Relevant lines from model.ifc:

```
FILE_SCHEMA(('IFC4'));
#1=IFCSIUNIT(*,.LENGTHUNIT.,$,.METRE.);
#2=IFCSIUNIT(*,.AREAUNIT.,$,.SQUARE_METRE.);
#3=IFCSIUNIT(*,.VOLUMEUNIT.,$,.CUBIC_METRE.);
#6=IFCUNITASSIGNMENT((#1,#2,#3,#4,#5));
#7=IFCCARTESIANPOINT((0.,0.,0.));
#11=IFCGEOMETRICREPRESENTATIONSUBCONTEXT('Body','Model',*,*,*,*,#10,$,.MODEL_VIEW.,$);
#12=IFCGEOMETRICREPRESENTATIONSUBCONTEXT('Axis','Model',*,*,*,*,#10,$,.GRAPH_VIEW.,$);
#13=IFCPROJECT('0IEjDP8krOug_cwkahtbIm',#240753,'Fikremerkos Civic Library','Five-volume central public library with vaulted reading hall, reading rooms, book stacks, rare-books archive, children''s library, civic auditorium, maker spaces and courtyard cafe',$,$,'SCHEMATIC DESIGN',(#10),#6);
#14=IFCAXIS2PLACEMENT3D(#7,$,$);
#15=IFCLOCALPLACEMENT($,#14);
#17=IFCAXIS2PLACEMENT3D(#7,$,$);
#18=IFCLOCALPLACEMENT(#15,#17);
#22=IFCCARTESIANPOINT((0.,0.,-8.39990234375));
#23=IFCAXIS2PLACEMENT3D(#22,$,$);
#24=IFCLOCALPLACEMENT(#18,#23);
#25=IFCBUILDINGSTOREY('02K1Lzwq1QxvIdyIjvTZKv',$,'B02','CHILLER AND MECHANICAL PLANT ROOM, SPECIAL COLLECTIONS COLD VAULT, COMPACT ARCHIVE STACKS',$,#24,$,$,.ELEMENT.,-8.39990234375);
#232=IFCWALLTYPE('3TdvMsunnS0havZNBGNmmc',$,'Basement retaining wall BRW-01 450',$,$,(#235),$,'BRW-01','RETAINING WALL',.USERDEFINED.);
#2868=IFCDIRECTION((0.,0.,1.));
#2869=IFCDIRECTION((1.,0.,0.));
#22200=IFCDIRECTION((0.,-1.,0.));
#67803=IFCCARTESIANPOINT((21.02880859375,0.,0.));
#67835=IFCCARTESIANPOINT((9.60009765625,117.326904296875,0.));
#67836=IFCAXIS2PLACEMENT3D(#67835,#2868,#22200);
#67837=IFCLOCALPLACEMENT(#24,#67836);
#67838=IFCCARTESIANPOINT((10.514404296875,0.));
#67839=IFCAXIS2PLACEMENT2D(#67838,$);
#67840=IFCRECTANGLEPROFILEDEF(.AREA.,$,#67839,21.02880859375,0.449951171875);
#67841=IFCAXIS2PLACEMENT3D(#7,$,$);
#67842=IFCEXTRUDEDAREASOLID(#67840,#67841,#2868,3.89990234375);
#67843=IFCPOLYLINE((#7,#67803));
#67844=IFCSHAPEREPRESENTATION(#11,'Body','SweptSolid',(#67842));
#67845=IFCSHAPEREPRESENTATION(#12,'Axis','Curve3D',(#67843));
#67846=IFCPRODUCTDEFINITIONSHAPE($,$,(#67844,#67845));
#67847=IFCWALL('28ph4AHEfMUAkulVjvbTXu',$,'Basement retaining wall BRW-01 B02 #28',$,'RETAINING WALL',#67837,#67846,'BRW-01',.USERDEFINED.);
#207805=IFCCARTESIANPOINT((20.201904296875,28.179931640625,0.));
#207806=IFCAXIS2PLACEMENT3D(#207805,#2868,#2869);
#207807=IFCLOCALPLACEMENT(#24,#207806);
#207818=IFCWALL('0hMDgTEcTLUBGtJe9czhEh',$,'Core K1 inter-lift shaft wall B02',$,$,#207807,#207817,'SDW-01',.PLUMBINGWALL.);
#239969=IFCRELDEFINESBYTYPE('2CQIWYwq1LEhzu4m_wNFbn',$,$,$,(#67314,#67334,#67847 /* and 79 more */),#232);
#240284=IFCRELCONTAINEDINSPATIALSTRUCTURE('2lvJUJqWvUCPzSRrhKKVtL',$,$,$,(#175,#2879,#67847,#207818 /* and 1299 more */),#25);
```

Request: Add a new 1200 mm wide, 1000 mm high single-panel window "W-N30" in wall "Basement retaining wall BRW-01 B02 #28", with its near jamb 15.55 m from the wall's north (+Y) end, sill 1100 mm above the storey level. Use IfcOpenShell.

```python
import numpy as np
import ifcopenshell
import ifcopenshell.api.feature
import ifcopenshell.api.geometry
import ifcopenshell.api.root
import ifcopenshell.api.spatial
import ifcopenshell.geom
import ifcopenshell.util.element
import ifcopenshell.util.placement
import ifcopenshell.util.representation
import ifcopenshell.util.shape
import ifcopenshell.util.unit

model = ifcopenshell.open("model.ifc")
unit_scale = ifcopenshell.util.unit.calculate_unit_scale(model)
settings = ifcopenshell.geom.settings()


def volume(element):
    """Net volume in cubic metres, openings subtracted."""
    shape = ifcopenshell.geom.create_shape(settings, element)
    return ifcopenshell.util.shape.get_volume(shape.geometry)


wall = model.by_guid("28ph4AHEfMUAkulVjvbTXu")
storey = ifcopenshell.util.element.get_container(wall, ifc_class="IfcBuildingStorey")
context = ifcopenshell.util.representation.get_context(model, "Model", "Body", "MODEL_VIEW")
before = volume(wall)

width, height, from_end, sill = 1.2, 1, 15.55, 1.1  # metres

# The wall runs along its own X axis, and the end named is its -X end.
wall_shape = ifcopenshell.geom.create_shape(settings, wall)
x, y, z = ifcopenshell.util.shape.get_vertices(wall_shape.geometry).T
start = x.min() + from_end
face, thickness = float(y.min()), float(y.max() - y.min())
wall_matrix = ifcopenshell.util.placement.get_local_placement(wall.ObjectPlacement)
level = ifcopenshell.util.placement.get_local_placement(storey.ObjectPlacement)[2, 3]


def in_wall(x, y):
    """Placement at x, y metres in the wall's axes, at sill height."""
    matrix = wall_matrix.copy()
    matrix[:, 3] = wall_matrix @ np.array([x / unit_scale, y / unit_scale, 0.0, 1.0])
    matrix[2, 3] = level + sill / unit_scale
    return matrix


# Opening: a box that overshoots both wall faces by 50 mm.
opening = ifcopenshell.api.root.create_entity(model, ifc_class="IfcOpeningElement", predefined_type="OPENING")
box = ifcopenshell.api.geometry.add_wall_representation(
    model, context=context, length=width, height=height, thickness=thickness + 0.1
)
ifcopenshell.api.geometry.assign_representation(model, product=opening, representation=box)
ifcopenshell.api.geometry.edit_object_placement(model, product=opening, matrix=in_wall(start, face - 0.05), is_si=False)
ifcopenshell.api.feature.add_feature(model, feature=opening, element=wall)

window = ifcopenshell.api.root.create_entity(model, ifc_class="IfcWindow", name="W-N30", predefined_type="WINDOW")
window.OverallWidth, window.OverallHeight = width / unit_scale, height / unit_scale
window.PartitioningType = "SINGLE_PANEL"
body = ifcopenshell.api.geometry.add_window_representation(
    model,
    context=context,
    overall_width=window.OverallWidth,
    overall_height=window.OverallHeight,
    partition_type="SINGLE_PANEL",
)
ifcopenshell.api.geometry.assign_representation(model, product=window, representation=body)
ifcopenshell.api.spatial.assign_container(model, products=[window], relating_structure=storey)
ifcopenshell.api.feature.add_filling(model, opening=opening, element=window)

# Centre the window in the wall's thickness.
ifcopenshell.api.geometry.edit_object_placement(model, product=window, matrix=in_wall(start, face), is_si=False)
window_shape = ifcopenshell.geom.create_shape(settings, window)
depth = ifcopenshell.util.shape.get_vertices(window_shape.geometry)[:, 1]
offset = face + thickness / 2 - (depth.min() + depth.max()) / 2
ifcopenshell.api.geometry.edit_object_placement(model, product=window, matrix=in_wall(start, offset), is_si=False)

after = volume(wall)

print(f"wall volume {before:.3f} -> {after:.3f} m3")

model.write("model-out.ifc")
```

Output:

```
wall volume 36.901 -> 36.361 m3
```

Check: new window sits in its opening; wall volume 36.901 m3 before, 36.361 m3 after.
